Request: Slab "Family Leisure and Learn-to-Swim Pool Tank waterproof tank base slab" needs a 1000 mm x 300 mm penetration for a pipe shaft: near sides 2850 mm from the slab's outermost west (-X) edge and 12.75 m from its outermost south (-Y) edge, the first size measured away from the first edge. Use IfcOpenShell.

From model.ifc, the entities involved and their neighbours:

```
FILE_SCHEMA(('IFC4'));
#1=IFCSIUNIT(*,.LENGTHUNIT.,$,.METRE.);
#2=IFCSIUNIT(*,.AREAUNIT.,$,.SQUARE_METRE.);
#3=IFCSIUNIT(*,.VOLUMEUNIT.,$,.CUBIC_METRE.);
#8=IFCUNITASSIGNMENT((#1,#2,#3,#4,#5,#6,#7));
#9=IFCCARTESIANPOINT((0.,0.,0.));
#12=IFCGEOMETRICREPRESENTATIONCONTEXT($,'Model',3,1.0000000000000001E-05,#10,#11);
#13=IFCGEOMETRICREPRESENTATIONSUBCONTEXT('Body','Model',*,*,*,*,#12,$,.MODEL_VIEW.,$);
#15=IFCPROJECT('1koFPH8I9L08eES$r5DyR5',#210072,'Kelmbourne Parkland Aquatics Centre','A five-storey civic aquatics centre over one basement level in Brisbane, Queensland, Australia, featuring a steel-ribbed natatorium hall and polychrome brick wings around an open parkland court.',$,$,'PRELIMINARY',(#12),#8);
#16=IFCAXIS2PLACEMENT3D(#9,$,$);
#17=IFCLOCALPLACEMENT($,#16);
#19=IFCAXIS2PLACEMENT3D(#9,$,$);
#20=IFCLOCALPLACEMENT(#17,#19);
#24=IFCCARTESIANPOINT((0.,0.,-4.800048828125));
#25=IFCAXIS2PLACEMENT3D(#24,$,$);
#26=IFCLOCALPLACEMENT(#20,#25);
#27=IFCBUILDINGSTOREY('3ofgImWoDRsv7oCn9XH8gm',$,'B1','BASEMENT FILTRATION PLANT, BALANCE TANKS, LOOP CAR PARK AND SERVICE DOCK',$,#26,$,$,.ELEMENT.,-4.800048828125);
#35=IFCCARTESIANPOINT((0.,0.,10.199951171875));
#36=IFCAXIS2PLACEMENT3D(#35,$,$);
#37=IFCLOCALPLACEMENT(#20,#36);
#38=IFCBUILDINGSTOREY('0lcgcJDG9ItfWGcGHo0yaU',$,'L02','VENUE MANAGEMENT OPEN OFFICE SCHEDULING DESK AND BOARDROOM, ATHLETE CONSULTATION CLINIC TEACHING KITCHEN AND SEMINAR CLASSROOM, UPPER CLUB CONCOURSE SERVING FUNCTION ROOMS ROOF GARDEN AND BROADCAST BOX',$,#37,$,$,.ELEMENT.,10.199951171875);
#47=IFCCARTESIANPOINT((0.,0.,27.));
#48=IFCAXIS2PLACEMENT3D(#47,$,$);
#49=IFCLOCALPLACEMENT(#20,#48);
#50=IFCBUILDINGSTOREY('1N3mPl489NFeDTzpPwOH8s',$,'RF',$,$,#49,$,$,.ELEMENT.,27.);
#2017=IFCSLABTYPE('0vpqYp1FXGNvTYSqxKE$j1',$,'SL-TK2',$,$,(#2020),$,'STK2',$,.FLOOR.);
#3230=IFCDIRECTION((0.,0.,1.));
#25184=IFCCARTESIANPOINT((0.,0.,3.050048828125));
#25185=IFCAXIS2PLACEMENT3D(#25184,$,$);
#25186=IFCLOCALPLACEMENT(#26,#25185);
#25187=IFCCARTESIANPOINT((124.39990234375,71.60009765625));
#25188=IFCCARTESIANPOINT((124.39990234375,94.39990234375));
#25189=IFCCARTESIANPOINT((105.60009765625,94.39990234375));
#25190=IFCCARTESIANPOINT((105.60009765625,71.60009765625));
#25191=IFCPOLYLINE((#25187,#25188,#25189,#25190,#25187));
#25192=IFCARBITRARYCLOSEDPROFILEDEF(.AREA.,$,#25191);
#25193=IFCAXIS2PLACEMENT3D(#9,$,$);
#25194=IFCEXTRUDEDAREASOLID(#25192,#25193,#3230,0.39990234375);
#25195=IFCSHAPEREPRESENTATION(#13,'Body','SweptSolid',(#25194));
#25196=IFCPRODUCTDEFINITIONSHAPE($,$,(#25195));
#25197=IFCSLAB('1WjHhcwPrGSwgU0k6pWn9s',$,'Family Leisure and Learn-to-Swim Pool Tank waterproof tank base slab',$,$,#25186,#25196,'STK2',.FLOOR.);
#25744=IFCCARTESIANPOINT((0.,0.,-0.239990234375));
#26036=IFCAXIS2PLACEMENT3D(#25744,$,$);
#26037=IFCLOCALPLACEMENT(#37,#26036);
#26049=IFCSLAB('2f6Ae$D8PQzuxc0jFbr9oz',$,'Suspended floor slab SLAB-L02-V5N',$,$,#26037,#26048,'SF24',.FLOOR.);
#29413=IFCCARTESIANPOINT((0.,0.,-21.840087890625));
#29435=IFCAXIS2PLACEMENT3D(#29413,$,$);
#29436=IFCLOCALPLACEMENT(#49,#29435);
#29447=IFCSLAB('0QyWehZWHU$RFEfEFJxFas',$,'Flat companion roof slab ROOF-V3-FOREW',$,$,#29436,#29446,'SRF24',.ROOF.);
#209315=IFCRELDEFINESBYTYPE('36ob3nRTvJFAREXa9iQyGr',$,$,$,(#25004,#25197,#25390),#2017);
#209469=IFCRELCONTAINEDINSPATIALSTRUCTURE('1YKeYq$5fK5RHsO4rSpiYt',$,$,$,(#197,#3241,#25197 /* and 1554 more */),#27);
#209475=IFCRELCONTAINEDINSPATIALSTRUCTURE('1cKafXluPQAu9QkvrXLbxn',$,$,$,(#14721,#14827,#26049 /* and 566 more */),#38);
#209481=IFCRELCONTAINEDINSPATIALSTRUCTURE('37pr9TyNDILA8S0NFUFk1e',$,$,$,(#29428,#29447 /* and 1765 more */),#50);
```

```python
import numpy as np
import ifcopenshell
import ifcopenshell.api.feature
import ifcopenshell.api.geometry
import ifcopenshell.api.root
import ifcopenshell.geom
import ifcopenshell.util.placement
import ifcopenshell.util.representation
import ifcopenshell.util.shape
import ifcopenshell.util.unit

model = ifcopenshell.open("model.ifc")
unit_scale = ifcopenshell.util.unit.calculate_unit_scale(model)
settings = ifcopenshell.geom.settings()


def volume(element):
    """Net volume in cubic metres, openings subtracted."""
    shape = ifcopenshell.geom.create_shape(settings, element)
    return ifcopenshell.util.shape.get_volume(shape.geometry)


slab = model.by_guid("1WjHhcwPrGSwgU0k6pWn9s")
before = volume(slab)

# Extent in the slab's own axes, in metres. The edges named are its -X and -Y sides.
slab_shape = ifcopenshell.geom.create_shape(settings, slab)
vertices = ifcopenshell.util.shape.get_vertices(slab_shape.geometry)
x_min, y_min, bottom = vertices.min(axis=0)
top = vertices[:, 2].max()

opening = ifcopenshell.api.root.create_entity(model, ifc_class="IfcOpeningElement", name="Pipe shaft opening", predefined_type="OPENING")
context = ifcopenshell.util.representation.get_context(model, "Model", "Body", "MODEL_VIEW")
width, depth = 1, 0.3
outline = [(0.0, 0.0), (width, 0.0), (width, depth), (0.0, depth), (0.0, 0.0)]
# Overshoot both faces by 50 mm so the cut is clean.
shape = ifcopenshell.api.geometry.add_slab_representation(
    model, context=context, depth=top - bottom + 0.1, polyline=outline
)
ifcopenshell.api.geometry.assign_representation(model, product=opening, representation=shape)

matrix = ifcopenshell.util.placement.get_local_placement(slab.ObjectPlacement)
matrix[:, 3] = matrix @ np.append(np.array([x_min + 2.85, y_min + 12.75, bottom - 0.05]) / unit_scale, 1.0)
ifcopenshell.api.geometry.edit_object_placement(model, product=opening, matrix=matrix, is_si=False)
ifcopenshell.api.feature.add_feature(model, feature=opening, element=slab)

after = volume(slab)

print(f"slab volume {before:.3f} -> {after:.3f} m3")

model.write("model_edited.ifc")
```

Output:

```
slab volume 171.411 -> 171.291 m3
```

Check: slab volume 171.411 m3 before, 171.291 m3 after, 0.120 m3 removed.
